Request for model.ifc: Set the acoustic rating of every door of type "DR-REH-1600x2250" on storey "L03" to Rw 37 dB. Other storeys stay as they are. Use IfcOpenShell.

First a look at what the model holds.

```python
import ifcopenshell
import ifcopenshell.util.element

model = ifcopenshell.open("model.ifc")
print(model.schema)
storey = next(s for s in model.by_type("IfcBuildingStorey") if s.Name == "L03")
doors = [e for e in ifcopenshell.util.element.get_decomposition(storey) if e.is_a("IfcDoor")]
seen = {}
for e in doors:
    element_type = ifcopenshell.util.element.get_type(e)
    key = (element_type.Name if element_type != e and element_type else None, ifcopenshell.util.element.get_pset(e, "Pset_DoorCommon", "AcousticRating"))
    seen[key] = seen.get(key, 0) + 1
for (name, value), count in sorted(seen.items(), key=str):
    print(count, "x", name, "|", value)
```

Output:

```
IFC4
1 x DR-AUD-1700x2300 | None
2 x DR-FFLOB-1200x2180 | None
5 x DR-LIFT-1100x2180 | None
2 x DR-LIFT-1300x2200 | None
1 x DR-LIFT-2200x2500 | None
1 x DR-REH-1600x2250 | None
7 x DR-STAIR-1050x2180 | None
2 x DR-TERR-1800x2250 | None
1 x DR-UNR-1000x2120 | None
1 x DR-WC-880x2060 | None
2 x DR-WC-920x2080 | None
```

```python
import ifcopenshell
import ifcopenshell.api.pset
import ifcopenshell.util.element

model = ifcopenshell.open("model.ifc")

storey = next(s for s in model.by_type("IfcBuildingStorey") if s.Name == "L03")
doors = [e for e in ifcopenshell.util.element.get_decomposition(storey) if e.is_a("IfcDoor")]

count = 0
for e in doors:
    element_type = ifcopenshell.util.element.get_type(e)
    if element_type in (None, e) or element_type.Name != "DR-REH-1600x2250":
        continue
    # add_pset returns the element's existing set when there is one.
    pset = ifcopenshell.api.pset.add_pset(model, product=e, name="Pset_DoorCommon")
    ifcopenshell.api.pset.edit_pset(model, pset=pset, properties={"AcousticRating": "Rw 37 dB"})
    count += 1

print(count, "doors updated")

model.write("model_updated.ifc")
```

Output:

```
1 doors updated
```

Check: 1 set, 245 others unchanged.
